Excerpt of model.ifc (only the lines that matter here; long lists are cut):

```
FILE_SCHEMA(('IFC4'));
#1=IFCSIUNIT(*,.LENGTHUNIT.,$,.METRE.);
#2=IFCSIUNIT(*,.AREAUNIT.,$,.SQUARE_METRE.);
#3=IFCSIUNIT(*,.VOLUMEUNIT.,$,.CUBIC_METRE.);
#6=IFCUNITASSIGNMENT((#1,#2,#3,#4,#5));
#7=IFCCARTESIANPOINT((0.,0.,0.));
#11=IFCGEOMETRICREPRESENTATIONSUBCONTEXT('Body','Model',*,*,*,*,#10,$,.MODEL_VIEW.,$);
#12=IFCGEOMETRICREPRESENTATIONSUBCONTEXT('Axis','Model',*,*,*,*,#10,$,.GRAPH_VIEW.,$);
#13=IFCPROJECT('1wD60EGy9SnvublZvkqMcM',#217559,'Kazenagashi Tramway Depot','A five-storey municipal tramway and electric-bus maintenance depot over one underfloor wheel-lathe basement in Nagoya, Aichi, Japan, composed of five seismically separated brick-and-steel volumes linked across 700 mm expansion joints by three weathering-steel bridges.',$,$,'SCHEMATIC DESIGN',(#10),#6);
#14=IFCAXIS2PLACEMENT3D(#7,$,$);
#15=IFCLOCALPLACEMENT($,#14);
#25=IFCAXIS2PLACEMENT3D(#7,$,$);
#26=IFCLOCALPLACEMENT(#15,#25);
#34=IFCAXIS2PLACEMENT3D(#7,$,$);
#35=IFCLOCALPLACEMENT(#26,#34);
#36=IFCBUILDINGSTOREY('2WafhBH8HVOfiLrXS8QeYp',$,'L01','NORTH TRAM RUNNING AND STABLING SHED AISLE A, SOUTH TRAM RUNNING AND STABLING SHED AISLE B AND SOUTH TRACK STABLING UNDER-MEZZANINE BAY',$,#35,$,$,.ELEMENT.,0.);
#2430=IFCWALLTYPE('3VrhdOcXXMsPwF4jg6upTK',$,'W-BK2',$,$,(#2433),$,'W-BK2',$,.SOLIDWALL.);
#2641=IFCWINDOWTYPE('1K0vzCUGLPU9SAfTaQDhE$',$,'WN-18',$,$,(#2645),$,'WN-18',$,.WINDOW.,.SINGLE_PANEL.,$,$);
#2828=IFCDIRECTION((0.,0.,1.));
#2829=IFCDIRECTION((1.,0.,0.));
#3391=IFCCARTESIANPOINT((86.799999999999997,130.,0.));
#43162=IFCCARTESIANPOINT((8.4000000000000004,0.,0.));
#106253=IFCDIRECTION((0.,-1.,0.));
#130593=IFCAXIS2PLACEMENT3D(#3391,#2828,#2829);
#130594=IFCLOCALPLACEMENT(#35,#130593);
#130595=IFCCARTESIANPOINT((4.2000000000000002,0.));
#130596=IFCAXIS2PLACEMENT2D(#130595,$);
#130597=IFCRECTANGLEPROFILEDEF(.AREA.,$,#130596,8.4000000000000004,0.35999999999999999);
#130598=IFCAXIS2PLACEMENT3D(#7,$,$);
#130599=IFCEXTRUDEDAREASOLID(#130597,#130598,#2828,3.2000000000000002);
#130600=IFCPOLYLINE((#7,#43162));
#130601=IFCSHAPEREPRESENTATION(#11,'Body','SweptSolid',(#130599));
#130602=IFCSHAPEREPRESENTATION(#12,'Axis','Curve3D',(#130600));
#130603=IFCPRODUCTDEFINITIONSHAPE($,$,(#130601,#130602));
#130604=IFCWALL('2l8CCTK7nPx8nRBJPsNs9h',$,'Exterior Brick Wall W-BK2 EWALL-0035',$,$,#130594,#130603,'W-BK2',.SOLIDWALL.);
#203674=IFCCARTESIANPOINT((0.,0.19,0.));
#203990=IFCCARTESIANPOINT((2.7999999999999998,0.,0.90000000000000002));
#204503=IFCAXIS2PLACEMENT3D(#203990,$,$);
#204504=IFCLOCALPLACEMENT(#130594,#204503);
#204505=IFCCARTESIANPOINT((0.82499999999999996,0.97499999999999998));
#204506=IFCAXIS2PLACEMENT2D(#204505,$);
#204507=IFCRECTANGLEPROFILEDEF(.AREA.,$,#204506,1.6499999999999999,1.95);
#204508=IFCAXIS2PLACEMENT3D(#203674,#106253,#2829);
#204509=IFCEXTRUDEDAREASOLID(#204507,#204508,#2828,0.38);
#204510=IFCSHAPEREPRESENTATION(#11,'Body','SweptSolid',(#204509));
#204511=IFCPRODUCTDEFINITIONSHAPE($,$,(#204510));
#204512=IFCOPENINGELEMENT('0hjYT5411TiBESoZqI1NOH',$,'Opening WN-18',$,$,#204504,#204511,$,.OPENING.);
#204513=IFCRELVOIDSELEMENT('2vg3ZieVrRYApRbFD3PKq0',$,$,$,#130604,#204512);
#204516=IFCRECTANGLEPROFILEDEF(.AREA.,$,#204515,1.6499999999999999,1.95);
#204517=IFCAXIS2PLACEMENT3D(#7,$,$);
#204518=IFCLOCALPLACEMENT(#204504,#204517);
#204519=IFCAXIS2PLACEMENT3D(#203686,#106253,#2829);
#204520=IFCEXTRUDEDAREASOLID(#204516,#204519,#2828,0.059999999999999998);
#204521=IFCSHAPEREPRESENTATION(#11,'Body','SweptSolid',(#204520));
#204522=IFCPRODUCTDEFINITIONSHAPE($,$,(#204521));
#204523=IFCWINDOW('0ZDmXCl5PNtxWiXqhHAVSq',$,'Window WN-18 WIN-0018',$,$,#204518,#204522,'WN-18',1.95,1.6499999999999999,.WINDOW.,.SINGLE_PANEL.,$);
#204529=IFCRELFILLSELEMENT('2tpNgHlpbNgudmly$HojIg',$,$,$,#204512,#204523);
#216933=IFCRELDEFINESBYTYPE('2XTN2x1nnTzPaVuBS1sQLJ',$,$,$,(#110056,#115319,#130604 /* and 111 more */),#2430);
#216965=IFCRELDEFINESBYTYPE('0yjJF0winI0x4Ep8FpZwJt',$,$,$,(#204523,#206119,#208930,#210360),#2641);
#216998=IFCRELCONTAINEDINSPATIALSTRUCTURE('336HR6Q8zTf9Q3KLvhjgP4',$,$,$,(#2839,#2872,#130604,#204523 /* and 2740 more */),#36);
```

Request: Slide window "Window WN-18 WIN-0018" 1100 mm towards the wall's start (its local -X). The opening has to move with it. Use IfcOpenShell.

```python
import ifcopenshell
import ifcopenshell.api.geometry
import ifcopenshell.util.placement
import ifcopenshell.util.unit

model = ifcopenshell.open("model.ifc")
unit_scale = ifcopenshell.util.unit.calculate_unit_scale(model)

window = model.by_guid("0ZDmXCl5PNtxWiXqhHAVSq")
opening = window.FillsVoids[0].RelatingOpeningElement
wall = opening.VoidsElements[0].RelatingBuildingElement

wall_matrix = ifcopenshell.util.placement.get_local_placement(wall.ObjectPlacement)
shift = wall_matrix[:3, 0] * -1.1 / unit_scale
before = ifcopenshell.util.placement.get_local_placement(window.ObjectPlacement)[:3, 3].copy()

# The window is placed relative to its opening, so it follows when the opening moves.
matrix = ifcopenshell.util.placement.get_local_placement(opening.ObjectPlacement)
matrix[:3, 3] += shift
ifcopenshell.api.geometry.edit_object_placement(
    model, product=opening, matrix=matrix, is_si=False, should_transform_children=True
)

after = ifcopenshell.util.placement.get_local_placement(window.ObjectPlacement)[:3, 3]
print("window moved by", (after - before).round(3) + 0.0)

model.write("model-out.ifc")
```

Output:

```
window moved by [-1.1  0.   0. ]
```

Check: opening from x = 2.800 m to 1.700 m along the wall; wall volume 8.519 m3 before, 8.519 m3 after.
